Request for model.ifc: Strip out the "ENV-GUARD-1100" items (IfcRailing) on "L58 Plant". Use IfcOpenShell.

First a look at what the model holds.

```python
import ifcopenshell
import ifcopenshell.util.element

model = ifcopenshell.open("model.ifc")
print(model.schema)
storey = next(s for s in model.by_type("IfcBuildingStorey") if s.Name == "L58 Plant")
railings = [e for e in ifcopenshell.util.element.get_decomposition(storey) if e.is_a("IfcRailing")]
seen = {}
for e in railings:
    element_type = ifcopenshell.util.element.get_type(e)
    name = element_type.Name if element_type not in (None, e) else None
    seen[name] = seen.get(name, 0) + 1
for name, count in sorted(seen.items(), key=str):
    print(count, "x", name)
```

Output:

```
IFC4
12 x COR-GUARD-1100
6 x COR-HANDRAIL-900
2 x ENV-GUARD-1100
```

```python
import ifcopenshell
import ifcopenshell.api.root
import ifcopenshell.util.element

model = ifcopenshell.open("model.ifc")

storey = next(s for s in model.by_type("IfcBuildingStorey") if s.Name == "L58 Plant")
railings = [e for e in ifcopenshell.util.element.get_decomposition(storey) if e.is_a("IfcRailing")]
targets = [e for e in railings if (t := ifcopenshell.util.element.get_type(e)) not in (None, e) and t.Name == "ENV-GUARD-1100"]

for e in targets:
    ifcopenshell.api.root.remove_product(model, product=e)
print(len(targets), "removed")

model.write("model_updated.ifc")
```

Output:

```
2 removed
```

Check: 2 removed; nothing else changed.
